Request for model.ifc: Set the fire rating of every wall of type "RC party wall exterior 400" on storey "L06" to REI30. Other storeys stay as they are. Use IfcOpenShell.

First a look at what the model holds.

```python
import ifcopenshell
import ifcopenshell.util.element

model = ifcopenshell.open("model.ifc")
print(model.schema)
storey = next(s for s in model.by_type("IfcBuildingStorey") if s.Name == "L06")
walls = [e for e in ifcopenshell.util.element.get_decomposition(storey) if e.is_a("IfcWall")]
seen = {}
for e in walls:
    element_type = ifcopenshell.util.element.get_type(e)
    key = (element_type.Name if element_type != e and element_type else None, ifcopenshell.util.element.get_pset(e, "Pset_WallCommon", "FireRating"))
    seen[key] = seen.get(key, 0) + 1
for (name, value), count in sorted(seen.items(), key=str):
    print(count, "x", name, "|", value)
```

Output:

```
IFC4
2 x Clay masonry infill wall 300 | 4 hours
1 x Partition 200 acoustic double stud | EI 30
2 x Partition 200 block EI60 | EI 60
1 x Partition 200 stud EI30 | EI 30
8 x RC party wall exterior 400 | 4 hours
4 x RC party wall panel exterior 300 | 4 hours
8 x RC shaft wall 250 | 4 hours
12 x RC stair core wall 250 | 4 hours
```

```python
import ifcopenshell
import ifcopenshell.api.pset
import ifcopenshell.util.element

model = ifcopenshell.open("model.ifc")

storey = next(s for s in model.by_type("IfcBuildingStorey") if s.Name == "L06")
walls = [e for e in ifcopenshell.util.element.get_decomposition(storey) if e.is_a("IfcWall")]

count = 0
for e in walls:
    element_type = ifcopenshell.util.element.get_type(e)
    if element_type in (None, e) or element_type.Name != "RC party wall exterior 400":
        continue
    # add_pset returns the element's existing set when there is one.
    pset = ifcopenshell.api.pset.add_pset(model, product=e, name="Pset_WallCommon")
    ifcopenshell.api.pset.edit_pset(model, pset=pset, properties={"FireRating": "REI30"})
    count += 1

print(count, "walls updated")

model.write("model_updated.ifc")
```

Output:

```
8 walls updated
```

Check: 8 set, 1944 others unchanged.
